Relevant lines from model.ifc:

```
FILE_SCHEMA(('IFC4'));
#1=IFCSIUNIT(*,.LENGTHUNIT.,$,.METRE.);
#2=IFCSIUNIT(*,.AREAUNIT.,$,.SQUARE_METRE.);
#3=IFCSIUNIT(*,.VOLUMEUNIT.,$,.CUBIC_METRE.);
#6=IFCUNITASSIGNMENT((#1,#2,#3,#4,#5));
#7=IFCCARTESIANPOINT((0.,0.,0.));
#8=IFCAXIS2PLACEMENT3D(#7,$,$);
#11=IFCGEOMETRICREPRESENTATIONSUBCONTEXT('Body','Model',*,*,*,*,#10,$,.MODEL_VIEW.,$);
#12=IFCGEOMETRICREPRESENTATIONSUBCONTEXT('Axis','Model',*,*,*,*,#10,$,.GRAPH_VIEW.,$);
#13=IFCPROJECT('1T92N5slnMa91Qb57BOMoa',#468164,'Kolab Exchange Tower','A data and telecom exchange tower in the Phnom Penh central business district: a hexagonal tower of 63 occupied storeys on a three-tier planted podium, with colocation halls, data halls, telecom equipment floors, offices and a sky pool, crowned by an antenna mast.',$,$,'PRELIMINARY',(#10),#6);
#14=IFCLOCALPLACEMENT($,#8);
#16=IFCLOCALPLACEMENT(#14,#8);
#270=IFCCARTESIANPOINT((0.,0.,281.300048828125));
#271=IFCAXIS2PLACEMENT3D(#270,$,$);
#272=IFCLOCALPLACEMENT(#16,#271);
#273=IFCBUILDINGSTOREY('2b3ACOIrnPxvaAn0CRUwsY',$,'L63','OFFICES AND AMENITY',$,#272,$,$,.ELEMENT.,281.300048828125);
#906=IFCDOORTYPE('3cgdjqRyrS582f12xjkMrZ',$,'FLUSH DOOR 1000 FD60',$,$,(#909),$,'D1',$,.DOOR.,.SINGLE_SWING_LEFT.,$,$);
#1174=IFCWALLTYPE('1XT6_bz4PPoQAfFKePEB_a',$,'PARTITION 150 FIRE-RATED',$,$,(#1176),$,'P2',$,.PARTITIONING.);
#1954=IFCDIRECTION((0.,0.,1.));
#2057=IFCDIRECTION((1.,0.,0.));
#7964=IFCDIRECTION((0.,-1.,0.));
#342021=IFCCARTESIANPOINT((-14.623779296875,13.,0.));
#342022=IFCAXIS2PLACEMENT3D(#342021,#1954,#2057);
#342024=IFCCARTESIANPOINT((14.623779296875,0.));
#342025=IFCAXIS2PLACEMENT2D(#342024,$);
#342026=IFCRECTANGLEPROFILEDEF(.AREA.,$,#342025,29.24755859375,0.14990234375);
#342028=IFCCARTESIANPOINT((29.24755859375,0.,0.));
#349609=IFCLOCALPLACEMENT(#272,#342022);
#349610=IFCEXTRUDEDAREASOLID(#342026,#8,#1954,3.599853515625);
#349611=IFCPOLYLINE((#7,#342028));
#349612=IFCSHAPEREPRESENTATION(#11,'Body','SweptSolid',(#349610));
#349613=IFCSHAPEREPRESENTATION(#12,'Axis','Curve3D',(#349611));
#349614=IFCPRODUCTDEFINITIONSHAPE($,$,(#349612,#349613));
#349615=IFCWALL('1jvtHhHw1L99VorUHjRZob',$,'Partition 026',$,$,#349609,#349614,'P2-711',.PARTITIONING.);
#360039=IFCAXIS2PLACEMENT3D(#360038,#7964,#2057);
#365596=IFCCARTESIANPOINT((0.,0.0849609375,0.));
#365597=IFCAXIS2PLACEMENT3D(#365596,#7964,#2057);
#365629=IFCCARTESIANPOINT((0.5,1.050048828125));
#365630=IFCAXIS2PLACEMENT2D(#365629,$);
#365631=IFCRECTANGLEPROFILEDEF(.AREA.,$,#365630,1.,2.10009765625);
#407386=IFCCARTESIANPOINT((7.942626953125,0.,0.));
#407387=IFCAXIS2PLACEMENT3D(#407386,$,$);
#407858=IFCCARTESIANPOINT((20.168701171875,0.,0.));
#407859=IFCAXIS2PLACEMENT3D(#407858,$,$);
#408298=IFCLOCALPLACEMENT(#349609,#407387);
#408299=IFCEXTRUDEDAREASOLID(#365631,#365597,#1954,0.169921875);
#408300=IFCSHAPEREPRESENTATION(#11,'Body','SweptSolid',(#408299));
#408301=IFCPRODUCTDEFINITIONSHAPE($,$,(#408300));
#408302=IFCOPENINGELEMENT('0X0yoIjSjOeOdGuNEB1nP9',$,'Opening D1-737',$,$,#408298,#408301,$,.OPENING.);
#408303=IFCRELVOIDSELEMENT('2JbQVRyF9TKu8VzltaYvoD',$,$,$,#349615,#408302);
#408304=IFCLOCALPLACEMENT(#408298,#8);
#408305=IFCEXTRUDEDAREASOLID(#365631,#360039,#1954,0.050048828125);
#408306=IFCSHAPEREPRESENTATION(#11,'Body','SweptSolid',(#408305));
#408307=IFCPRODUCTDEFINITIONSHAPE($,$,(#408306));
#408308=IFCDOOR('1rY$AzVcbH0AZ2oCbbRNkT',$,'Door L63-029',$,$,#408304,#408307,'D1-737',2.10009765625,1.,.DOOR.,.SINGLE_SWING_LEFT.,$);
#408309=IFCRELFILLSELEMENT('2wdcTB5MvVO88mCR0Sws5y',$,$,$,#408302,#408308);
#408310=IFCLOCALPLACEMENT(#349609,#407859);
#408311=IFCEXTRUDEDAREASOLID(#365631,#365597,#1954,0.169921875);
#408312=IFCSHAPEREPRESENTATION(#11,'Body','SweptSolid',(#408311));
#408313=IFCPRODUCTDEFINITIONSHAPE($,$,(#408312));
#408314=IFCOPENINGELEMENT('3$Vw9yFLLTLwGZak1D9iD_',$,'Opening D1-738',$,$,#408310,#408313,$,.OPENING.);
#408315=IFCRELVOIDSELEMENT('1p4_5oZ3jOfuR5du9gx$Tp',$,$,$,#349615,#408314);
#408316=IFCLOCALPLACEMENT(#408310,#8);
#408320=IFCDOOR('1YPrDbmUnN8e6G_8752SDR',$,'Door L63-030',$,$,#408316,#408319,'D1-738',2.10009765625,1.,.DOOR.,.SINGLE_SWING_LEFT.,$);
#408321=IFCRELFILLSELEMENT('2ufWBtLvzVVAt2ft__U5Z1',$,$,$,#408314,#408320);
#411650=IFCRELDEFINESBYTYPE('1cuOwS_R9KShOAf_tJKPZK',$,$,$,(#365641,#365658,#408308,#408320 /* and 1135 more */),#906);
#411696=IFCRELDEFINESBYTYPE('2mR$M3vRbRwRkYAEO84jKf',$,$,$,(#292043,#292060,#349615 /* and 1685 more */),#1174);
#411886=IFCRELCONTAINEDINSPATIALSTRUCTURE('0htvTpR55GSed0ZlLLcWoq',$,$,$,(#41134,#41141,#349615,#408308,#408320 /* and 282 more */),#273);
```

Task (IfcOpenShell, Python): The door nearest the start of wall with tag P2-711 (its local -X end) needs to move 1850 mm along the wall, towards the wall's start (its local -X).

```python
import ifcopenshell
import ifcopenshell.api.geometry
import ifcopenshell.util.placement
import ifcopenshell.util.unit

model = ifcopenshell.open("model.ifc")
unit_scale = ifcopenshell.util.unit.calculate_unit_scale(model)

door = model.by_guid("1rY$AzVcbH0AZ2oCbbRNkT")
opening = door.FillsVoids[0].RelatingOpeningElement
wall = opening.VoidsElements[0].RelatingBuildingElement

wall_matrix = ifcopenshell.util.placement.get_local_placement(wall.ObjectPlacement)
shift = wall_matrix[:3, 0] * -1.85 / unit_scale
before = ifcopenshell.util.placement.get_local_placement(door.ObjectPlacement)[:3, 3].copy()

# The door is placed relative to its opening, so it follows when the opening moves.
matrix = ifcopenshell.util.placement.get_local_placement(opening.ObjectPlacement)
matrix[:3, 3] += shift
ifcopenshell.api.geometry.edit_object_placement(
    model, product=opening, matrix=matrix, is_si=False, should_transform_children=True
)

after = ifcopenshell.util.placement.get_local_placement(door.ObjectPlacement)[:3, 3]
print("door moved by", (after - before).round(3) + 0.0)

model.write("model_updated.ifc")
```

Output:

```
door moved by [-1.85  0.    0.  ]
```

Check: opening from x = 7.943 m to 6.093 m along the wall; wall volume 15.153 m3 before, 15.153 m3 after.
